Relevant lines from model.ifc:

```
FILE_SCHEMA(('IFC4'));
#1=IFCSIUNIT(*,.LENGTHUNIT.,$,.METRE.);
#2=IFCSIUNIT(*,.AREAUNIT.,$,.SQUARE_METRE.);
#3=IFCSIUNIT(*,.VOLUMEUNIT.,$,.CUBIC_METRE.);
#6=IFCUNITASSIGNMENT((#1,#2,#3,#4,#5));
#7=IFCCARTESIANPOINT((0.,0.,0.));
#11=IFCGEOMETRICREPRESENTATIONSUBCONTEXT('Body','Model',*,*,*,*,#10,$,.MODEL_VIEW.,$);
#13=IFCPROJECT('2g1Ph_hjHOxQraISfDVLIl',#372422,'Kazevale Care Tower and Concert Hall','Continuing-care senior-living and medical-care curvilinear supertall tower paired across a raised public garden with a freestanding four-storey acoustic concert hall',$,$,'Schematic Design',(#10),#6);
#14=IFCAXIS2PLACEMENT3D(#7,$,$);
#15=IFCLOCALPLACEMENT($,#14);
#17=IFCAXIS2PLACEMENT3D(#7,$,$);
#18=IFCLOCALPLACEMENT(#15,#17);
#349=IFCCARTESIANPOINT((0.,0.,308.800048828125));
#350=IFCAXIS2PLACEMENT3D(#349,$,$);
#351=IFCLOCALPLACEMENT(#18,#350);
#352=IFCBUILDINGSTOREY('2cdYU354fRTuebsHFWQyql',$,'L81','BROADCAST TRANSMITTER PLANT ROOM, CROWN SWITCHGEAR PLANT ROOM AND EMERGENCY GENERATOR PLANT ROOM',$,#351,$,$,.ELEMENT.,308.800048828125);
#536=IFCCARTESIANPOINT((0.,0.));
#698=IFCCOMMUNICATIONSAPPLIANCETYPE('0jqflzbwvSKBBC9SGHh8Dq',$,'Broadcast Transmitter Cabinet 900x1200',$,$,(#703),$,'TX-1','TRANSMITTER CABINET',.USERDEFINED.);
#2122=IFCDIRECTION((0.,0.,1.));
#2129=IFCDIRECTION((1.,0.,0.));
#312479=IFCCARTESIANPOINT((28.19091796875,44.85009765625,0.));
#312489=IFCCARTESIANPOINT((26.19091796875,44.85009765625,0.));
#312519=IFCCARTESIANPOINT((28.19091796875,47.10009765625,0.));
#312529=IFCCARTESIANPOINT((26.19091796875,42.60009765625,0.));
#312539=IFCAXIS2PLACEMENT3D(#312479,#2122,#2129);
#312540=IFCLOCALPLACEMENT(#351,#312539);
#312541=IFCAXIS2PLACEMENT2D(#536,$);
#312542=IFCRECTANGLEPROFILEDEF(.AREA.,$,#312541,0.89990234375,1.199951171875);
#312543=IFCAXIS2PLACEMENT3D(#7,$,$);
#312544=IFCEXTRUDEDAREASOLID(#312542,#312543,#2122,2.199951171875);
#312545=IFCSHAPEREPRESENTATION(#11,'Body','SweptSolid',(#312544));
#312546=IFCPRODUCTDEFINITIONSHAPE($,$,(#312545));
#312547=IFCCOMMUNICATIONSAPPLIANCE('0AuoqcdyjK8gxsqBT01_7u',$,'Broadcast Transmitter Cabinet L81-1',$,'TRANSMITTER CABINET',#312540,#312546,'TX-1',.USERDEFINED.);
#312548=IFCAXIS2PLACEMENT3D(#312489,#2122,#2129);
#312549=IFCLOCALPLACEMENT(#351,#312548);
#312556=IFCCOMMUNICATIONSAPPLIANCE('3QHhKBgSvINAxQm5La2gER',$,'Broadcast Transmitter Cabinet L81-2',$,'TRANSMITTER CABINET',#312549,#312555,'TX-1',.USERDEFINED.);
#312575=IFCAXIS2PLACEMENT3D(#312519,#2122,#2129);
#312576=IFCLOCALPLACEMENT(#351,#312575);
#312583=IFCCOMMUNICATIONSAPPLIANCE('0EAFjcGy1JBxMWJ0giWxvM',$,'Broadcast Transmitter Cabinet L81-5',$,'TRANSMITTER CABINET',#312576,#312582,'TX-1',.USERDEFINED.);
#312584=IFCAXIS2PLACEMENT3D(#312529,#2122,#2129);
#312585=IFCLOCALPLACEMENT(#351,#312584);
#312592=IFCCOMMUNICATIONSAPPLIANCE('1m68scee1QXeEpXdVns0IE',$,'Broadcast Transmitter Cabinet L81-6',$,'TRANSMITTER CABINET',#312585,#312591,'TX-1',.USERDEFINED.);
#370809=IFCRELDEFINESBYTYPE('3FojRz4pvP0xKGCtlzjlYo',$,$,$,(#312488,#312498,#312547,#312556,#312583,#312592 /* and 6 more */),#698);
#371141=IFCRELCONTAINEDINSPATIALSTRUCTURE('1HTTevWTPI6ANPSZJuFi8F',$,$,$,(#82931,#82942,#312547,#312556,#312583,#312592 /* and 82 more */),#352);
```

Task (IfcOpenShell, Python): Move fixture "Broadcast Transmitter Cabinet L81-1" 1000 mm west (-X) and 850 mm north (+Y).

```python
import ifcopenshell
import ifcopenshell.api.geometry
import ifcopenshell.util.placement
import ifcopenshell.util.unit

model = ifcopenshell.open("model.ifc")
unit_scale = ifcopenshell.util.unit.calculate_unit_scale(model)

item = model.by_guid("0AuoqcdyjK8gxsqBT01_7u")
matrix = ifcopenshell.util.placement.get_local_placement(item.ObjectPlacement)
matrix[0, 3] -= 1 / unit_scale
matrix[1, 3] += 0.85 / unit_scale
ifcopenshell.api.geometry.edit_object_placement(model, product=item, matrix=matrix, is_si=False)

print(ifcopenshell.util.placement.get_local_placement(item.ObjectPlacement).round(3) + 0.0)

model.write("model_updated.ifc")
```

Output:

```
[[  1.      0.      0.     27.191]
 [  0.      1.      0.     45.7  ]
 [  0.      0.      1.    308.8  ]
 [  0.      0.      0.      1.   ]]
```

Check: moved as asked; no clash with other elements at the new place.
